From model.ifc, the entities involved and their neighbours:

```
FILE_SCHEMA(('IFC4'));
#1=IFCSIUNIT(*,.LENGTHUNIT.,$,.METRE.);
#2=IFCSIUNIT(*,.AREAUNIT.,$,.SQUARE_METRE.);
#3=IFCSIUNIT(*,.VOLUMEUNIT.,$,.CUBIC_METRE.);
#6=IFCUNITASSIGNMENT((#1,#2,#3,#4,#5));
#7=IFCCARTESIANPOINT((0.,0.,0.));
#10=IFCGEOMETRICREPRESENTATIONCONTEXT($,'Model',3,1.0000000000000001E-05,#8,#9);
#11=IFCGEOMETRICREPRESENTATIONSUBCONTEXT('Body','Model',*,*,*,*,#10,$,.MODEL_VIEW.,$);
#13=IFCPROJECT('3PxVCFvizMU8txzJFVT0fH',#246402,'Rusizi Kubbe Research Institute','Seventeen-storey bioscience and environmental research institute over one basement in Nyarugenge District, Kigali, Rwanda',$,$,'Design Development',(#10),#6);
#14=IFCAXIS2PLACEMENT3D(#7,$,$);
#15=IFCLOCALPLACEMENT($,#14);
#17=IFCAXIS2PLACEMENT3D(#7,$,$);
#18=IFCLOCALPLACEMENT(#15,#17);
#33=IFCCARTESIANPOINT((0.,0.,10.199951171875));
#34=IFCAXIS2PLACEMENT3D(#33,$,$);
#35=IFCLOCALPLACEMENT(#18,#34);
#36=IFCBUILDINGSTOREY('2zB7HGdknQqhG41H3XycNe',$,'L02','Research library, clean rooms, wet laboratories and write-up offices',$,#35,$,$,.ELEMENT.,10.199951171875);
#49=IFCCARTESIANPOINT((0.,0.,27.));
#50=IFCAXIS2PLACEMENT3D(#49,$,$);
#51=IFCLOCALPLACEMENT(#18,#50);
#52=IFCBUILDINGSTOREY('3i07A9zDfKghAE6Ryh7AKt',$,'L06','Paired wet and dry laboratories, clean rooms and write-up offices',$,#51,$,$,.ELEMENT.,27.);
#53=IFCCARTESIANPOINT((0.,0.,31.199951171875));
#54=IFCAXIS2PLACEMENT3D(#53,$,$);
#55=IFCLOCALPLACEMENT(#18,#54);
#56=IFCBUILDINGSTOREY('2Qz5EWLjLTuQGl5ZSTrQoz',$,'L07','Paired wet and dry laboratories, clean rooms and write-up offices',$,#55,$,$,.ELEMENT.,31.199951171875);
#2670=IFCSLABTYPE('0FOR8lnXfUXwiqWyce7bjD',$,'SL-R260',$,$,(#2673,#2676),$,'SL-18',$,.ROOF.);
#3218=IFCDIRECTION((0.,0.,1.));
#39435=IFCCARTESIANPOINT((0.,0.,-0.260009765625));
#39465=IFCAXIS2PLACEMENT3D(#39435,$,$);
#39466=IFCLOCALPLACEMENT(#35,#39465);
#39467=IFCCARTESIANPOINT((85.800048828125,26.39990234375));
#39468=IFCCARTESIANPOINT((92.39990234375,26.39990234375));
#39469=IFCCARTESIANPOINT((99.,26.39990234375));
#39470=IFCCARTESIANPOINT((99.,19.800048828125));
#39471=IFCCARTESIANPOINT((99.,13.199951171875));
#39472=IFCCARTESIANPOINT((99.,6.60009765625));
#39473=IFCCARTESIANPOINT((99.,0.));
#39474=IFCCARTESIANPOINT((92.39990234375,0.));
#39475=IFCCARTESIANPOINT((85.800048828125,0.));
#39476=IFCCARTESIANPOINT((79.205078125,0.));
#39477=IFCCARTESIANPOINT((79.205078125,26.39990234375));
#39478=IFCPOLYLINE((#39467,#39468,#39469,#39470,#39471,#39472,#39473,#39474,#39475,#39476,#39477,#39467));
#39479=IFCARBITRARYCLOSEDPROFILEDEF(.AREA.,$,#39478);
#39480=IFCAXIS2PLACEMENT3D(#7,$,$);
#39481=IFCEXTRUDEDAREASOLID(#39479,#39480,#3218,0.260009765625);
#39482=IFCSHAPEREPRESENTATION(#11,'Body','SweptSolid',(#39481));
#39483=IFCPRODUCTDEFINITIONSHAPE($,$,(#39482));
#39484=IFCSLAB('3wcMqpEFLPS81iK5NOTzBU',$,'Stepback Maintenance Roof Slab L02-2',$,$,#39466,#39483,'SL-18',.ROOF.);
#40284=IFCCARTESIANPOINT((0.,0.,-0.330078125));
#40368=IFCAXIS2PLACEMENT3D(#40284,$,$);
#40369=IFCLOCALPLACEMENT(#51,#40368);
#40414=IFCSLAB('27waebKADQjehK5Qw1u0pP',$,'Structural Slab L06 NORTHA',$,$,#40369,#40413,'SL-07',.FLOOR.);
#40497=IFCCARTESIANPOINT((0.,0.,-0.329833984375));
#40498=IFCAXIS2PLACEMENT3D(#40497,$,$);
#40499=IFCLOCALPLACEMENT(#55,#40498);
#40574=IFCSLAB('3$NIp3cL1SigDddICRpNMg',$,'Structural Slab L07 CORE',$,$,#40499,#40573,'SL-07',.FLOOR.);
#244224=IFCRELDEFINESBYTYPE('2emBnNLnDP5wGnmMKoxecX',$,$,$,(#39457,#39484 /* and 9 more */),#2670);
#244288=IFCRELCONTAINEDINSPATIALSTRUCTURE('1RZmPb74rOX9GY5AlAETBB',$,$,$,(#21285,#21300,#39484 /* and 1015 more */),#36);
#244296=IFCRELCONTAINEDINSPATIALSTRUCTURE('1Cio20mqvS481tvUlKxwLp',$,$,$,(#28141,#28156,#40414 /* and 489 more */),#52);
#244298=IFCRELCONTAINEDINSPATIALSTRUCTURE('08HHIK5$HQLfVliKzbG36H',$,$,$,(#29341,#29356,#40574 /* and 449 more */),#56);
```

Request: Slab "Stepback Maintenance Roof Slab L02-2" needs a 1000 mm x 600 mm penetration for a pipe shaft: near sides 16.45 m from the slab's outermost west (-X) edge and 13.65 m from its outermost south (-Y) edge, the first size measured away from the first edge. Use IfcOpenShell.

```python
import numpy as np
import ifcopenshell
import ifcopenshell.api.feature
import ifcopenshell.api.geometry
import ifcopenshell.api.root
import ifcopenshell.geom
import ifcopenshell.util.placement
import ifcopenshell.util.representation
import ifcopenshell.util.shape
import ifcopenshell.util.unit

model = ifcopenshell.open("model.ifc")
unit_scale = ifcopenshell.util.unit.calculate_unit_scale(model)
settings = ifcopenshell.geom.settings()


def volume(element):
    """Net volume in cubic metres, openings subtracted."""
    shape = ifcopenshell.geom.create_shape(settings, element)
    return ifcopenshell.util.shape.get_volume(shape.geometry)


slab = model.by_id(39484)
before = volume(slab)

# Extent in the slab's own axes, in metres. The edges named are its -X and -Y sides.
slab_shape = ifcopenshell.geom.create_shape(settings, slab)
vertices = ifcopenshell.util.shape.get_vertices(slab_shape.geometry)
x_min, y_min, bottom = vertices.min(axis=0)
top = vertices[:, 2].max()

opening = ifcopenshell.api.root.create_entity(model, ifc_class="IfcOpeningElement", name="Pipe shaft opening", predefined_type="OPENING")
context = ifcopenshell.util.representation.get_context(model, "Model", "Body", "MODEL_VIEW")
width, depth = 1, 0.6
outline = [(0.0, 0.0), (width, 0.0), (width, depth), (0.0, depth), (0.0, 0.0)]
# Overshoot both faces by 50 mm so the cut is clean.
shape = ifcopenshell.api.geometry.add_slab_representation(
    model, context=context, depth=top - bottom + 0.1, polyline=outline
)
ifcopenshell.api.geometry.assign_representation(model, product=opening, representation=shape)

matrix = ifcopenshell.util.placement.get_local_placement(slab.ObjectPlacement)
matrix[:, 3] = matrix @ np.append(np.array([x_min + 16.45, y_min + 13.65, bottom - 0.05]) / unit_scale, 1.0)
ifcopenshell.api.geometry.edit_object_placement(model, product=opening, matrix=matrix, is_si=False)
ifcopenshell.api.feature.add_feature(model, feature=opening, element=slab)

after = volume(slab)

print(f"slab volume {before:.3f} -> {after:.3f} m3")

model.write("model_v2.ifc")
```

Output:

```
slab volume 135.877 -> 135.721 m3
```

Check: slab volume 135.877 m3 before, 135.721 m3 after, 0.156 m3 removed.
